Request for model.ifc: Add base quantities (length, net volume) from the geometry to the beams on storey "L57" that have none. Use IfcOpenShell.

First a look at what the model holds.

```python
import ifcopenshell
import ifcopenshell.util.element
import ifcopenshell.util.unit

model = ifcopenshell.open("model.ifc")
print(model.schema)
for unit_type in ("LENGTHUNIT", "AREAUNIT", "VOLUMEUNIT"):
    print(unit_type, ifcopenshell.util.unit.calculate_unit_scale(model, unit_type))
storey = next(s for s in model.by_type("IfcBuildingStorey") if s.Name == "L57")
beams = [e for e in ifcopenshell.util.element.get_decomposition(storey) if e.is_a("IfcBeam")]
for e in sorted(beams, key=lambda e: e.id()):
    print(e.id(), e.is_a(), e.Name, list(ifcopenshell.util.element.get_psets(e, qtos_only=True)), sep=" | ")
```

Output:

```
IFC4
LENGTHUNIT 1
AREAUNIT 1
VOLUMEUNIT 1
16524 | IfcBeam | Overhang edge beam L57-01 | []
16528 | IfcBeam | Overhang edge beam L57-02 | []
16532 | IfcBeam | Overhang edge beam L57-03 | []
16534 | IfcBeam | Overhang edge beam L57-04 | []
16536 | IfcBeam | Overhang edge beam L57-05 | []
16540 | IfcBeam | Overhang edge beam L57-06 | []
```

```python
import ifcopenshell
import ifcopenshell.api.pset
import ifcopenshell.geom
import ifcopenshell.util.element
import ifcopenshell.util.shape
import ifcopenshell.util.unit

model = ifcopenshell.open("model.ifc")
unit_scale = ifcopenshell.util.unit.calculate_unit_scale(model)
volume_scale = ifcopenshell.util.unit.calculate_unit_scale(model, "VOLUMEUNIT")
settings = ifcopenshell.geom.settings()

storey = next(s for s in model.by_type("IfcBuildingStorey") if s.Name == "L57")
beams = [e for e in ifcopenshell.util.element.get_decomposition(storey) if e.is_a("IfcBeam")]

for e in sorted(beams, key=lambda e: e.id()):
    if ifcopenshell.util.element.get_psets(e, qtos_only=True, should_inherit=False):
        continue
    # Geometry comes back in metres, in the element's own axes.
    shape = ifcopenshell.geom.create_shape(settings, e)
    values = {
        "Length": ifcopenshell.util.shape.get_max_xyz(shape.geometry) / unit_scale,
        "NetVolume": ifcopenshell.util.shape.get_volume(shape.geometry) / volume_scale,
    }
    qto = ifcopenshell.api.pset.add_qto(model, product=e, name="Qto_BeamBaseQuantities")
    ifcopenshell.api.pset.edit_qto(model, qto=qto, properties=values)
    print(e.id(), {k: round(v, 3) for k, v in values.items()})

model.write("model_v2.ifc")
```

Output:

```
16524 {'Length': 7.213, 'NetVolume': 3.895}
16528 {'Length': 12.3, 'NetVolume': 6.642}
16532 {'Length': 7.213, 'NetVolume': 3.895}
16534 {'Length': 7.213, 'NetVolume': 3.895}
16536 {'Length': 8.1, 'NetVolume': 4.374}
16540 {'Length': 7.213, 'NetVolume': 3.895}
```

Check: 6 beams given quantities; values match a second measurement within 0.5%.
